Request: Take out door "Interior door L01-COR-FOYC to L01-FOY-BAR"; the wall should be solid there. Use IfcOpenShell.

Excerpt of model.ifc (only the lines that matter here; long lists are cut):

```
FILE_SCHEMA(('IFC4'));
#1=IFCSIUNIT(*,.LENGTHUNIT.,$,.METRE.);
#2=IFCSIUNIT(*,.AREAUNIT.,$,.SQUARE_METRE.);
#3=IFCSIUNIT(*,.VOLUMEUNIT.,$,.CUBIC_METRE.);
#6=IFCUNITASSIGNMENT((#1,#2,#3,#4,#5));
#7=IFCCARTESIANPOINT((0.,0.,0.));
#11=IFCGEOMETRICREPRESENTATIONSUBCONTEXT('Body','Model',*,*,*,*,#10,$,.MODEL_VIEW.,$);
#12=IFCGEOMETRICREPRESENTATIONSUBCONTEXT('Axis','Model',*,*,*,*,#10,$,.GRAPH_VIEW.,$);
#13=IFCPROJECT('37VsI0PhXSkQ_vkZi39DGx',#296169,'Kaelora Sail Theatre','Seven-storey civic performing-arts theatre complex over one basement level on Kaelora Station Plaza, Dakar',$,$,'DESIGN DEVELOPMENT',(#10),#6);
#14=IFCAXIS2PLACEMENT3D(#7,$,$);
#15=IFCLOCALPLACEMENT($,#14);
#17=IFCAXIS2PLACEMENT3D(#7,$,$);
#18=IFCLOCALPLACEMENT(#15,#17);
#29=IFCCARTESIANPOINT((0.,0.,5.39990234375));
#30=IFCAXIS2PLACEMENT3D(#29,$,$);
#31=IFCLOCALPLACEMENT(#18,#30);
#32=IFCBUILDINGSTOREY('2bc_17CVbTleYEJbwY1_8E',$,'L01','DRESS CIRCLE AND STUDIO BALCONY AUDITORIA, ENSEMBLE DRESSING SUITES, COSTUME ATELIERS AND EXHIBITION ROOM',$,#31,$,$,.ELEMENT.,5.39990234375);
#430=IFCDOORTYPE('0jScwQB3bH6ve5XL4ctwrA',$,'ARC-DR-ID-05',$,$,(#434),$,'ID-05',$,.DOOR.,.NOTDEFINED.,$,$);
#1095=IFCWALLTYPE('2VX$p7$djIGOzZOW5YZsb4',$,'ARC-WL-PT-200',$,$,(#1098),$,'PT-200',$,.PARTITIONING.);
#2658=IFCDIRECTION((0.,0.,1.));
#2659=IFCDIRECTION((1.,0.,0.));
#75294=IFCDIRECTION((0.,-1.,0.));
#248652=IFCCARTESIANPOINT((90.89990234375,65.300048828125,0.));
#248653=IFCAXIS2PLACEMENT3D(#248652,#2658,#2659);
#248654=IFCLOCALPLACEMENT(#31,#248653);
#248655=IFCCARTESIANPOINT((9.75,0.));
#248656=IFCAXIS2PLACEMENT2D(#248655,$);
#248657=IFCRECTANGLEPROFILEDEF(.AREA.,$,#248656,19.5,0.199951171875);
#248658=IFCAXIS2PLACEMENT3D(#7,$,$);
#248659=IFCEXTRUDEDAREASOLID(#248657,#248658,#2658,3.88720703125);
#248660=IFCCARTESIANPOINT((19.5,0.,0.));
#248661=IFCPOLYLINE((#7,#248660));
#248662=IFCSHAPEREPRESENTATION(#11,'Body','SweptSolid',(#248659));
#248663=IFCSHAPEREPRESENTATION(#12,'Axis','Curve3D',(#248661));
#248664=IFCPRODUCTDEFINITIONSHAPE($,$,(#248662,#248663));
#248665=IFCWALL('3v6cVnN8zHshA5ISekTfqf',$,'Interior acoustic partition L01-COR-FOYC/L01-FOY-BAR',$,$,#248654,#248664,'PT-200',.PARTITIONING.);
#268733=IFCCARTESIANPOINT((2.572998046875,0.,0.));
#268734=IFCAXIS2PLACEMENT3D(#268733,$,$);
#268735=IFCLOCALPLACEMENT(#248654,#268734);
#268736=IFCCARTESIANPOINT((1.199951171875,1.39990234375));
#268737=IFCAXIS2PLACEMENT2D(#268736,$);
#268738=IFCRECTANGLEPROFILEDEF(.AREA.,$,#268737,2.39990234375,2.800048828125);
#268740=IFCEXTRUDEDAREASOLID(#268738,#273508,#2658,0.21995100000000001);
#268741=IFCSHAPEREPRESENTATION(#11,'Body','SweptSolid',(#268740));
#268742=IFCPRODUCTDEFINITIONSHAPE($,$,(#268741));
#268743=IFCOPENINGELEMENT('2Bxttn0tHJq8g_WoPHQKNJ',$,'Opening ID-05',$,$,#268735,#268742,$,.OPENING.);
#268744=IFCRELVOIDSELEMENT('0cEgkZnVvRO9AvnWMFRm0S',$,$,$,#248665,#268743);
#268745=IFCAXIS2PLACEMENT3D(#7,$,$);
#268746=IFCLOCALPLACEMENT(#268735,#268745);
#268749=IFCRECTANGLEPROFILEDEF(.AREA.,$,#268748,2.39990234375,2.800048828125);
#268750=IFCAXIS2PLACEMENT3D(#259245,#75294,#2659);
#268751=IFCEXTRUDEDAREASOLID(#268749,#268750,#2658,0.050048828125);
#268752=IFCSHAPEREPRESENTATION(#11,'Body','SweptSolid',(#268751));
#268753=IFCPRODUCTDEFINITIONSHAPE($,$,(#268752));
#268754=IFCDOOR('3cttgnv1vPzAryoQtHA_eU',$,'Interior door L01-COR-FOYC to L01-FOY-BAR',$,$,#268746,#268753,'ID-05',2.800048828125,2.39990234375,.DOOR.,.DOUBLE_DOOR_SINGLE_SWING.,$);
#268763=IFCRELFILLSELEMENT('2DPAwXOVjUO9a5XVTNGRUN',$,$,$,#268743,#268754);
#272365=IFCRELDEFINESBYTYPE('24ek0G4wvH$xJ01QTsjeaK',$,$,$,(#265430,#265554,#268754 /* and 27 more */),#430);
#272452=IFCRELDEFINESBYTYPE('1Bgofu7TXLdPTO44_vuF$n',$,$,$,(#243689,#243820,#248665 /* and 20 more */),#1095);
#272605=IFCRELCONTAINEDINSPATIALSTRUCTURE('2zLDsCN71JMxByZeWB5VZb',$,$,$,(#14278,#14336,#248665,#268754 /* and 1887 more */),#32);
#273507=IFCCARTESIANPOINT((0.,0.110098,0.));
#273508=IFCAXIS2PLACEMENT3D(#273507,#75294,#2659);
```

```python
import ifcopenshell
import ifcopenshell.api.feature
import ifcopenshell.api.root
import ifcopenshell.geom
import ifcopenshell.util.shape

model = ifcopenshell.open("model.ifc")
settings = ifcopenshell.geom.settings()


def volume(element):
    """Net volume in cubic metres, openings subtracted."""
    shape = ifcopenshell.geom.create_shape(settings, element)
    return ifcopenshell.util.shape.get_volume(shape.geometry)


door = model.by_guid("3cttgnv1vPzAryoQtHA_eU")
opening = door.FillsVoids[0].RelatingOpeningElement
wall = opening.VoidsElements[0].RelatingBuildingElement
before = volume(wall)

ifcopenshell.api.root.remove_product(model, product=door)
ifcopenshell.api.feature.remove_feature(model, feature=opening)

after = volume(wall)

print(f"wall volume {before:.3f} -> {after:.3f} m3")

model.write("model_rev.ifc")
```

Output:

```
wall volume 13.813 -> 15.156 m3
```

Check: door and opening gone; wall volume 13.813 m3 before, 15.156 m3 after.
